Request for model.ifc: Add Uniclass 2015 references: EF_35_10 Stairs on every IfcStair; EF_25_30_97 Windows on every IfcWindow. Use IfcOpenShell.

First a look at what the model holds.

```python
import ifcopenshell

model = ifcopenshell.open("model.ifc")
print(model.schema)
print("classifications:", [c.Name for c in model.by_type("IfcClassification")])
for ifc_class in ("IfcDoor", "IfcRoof", "IfcStair", "IfcWall", "IfcWindow"):
    print(ifc_class, len(model.by_type(ifc_class)))
```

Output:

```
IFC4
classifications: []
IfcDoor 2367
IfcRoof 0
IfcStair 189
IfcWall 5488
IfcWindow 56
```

```python
import ifcopenshell
import ifcopenshell.api.classification

model = ifcopenshell.open("model.ifc")

system = ifcopenshell.api.classification.add_classification(model, classification="Uniclass 2015")

codes = {
    "IfcStair": ("EF_35_10", "Stairs"),
    "IfcWindow": ("EF_25_30_97", "Windows"),
}
for ifc_class, (code, name) in codes.items():
    products = model.by_type(ifc_class)
    ifcopenshell.api.classification.add_reference(
        model, products=products, classification=system, identification=code, name=name
    )
    print(code, len(products))

model.write("model_edited.ifc")
```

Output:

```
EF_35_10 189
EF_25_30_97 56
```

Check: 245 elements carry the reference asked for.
